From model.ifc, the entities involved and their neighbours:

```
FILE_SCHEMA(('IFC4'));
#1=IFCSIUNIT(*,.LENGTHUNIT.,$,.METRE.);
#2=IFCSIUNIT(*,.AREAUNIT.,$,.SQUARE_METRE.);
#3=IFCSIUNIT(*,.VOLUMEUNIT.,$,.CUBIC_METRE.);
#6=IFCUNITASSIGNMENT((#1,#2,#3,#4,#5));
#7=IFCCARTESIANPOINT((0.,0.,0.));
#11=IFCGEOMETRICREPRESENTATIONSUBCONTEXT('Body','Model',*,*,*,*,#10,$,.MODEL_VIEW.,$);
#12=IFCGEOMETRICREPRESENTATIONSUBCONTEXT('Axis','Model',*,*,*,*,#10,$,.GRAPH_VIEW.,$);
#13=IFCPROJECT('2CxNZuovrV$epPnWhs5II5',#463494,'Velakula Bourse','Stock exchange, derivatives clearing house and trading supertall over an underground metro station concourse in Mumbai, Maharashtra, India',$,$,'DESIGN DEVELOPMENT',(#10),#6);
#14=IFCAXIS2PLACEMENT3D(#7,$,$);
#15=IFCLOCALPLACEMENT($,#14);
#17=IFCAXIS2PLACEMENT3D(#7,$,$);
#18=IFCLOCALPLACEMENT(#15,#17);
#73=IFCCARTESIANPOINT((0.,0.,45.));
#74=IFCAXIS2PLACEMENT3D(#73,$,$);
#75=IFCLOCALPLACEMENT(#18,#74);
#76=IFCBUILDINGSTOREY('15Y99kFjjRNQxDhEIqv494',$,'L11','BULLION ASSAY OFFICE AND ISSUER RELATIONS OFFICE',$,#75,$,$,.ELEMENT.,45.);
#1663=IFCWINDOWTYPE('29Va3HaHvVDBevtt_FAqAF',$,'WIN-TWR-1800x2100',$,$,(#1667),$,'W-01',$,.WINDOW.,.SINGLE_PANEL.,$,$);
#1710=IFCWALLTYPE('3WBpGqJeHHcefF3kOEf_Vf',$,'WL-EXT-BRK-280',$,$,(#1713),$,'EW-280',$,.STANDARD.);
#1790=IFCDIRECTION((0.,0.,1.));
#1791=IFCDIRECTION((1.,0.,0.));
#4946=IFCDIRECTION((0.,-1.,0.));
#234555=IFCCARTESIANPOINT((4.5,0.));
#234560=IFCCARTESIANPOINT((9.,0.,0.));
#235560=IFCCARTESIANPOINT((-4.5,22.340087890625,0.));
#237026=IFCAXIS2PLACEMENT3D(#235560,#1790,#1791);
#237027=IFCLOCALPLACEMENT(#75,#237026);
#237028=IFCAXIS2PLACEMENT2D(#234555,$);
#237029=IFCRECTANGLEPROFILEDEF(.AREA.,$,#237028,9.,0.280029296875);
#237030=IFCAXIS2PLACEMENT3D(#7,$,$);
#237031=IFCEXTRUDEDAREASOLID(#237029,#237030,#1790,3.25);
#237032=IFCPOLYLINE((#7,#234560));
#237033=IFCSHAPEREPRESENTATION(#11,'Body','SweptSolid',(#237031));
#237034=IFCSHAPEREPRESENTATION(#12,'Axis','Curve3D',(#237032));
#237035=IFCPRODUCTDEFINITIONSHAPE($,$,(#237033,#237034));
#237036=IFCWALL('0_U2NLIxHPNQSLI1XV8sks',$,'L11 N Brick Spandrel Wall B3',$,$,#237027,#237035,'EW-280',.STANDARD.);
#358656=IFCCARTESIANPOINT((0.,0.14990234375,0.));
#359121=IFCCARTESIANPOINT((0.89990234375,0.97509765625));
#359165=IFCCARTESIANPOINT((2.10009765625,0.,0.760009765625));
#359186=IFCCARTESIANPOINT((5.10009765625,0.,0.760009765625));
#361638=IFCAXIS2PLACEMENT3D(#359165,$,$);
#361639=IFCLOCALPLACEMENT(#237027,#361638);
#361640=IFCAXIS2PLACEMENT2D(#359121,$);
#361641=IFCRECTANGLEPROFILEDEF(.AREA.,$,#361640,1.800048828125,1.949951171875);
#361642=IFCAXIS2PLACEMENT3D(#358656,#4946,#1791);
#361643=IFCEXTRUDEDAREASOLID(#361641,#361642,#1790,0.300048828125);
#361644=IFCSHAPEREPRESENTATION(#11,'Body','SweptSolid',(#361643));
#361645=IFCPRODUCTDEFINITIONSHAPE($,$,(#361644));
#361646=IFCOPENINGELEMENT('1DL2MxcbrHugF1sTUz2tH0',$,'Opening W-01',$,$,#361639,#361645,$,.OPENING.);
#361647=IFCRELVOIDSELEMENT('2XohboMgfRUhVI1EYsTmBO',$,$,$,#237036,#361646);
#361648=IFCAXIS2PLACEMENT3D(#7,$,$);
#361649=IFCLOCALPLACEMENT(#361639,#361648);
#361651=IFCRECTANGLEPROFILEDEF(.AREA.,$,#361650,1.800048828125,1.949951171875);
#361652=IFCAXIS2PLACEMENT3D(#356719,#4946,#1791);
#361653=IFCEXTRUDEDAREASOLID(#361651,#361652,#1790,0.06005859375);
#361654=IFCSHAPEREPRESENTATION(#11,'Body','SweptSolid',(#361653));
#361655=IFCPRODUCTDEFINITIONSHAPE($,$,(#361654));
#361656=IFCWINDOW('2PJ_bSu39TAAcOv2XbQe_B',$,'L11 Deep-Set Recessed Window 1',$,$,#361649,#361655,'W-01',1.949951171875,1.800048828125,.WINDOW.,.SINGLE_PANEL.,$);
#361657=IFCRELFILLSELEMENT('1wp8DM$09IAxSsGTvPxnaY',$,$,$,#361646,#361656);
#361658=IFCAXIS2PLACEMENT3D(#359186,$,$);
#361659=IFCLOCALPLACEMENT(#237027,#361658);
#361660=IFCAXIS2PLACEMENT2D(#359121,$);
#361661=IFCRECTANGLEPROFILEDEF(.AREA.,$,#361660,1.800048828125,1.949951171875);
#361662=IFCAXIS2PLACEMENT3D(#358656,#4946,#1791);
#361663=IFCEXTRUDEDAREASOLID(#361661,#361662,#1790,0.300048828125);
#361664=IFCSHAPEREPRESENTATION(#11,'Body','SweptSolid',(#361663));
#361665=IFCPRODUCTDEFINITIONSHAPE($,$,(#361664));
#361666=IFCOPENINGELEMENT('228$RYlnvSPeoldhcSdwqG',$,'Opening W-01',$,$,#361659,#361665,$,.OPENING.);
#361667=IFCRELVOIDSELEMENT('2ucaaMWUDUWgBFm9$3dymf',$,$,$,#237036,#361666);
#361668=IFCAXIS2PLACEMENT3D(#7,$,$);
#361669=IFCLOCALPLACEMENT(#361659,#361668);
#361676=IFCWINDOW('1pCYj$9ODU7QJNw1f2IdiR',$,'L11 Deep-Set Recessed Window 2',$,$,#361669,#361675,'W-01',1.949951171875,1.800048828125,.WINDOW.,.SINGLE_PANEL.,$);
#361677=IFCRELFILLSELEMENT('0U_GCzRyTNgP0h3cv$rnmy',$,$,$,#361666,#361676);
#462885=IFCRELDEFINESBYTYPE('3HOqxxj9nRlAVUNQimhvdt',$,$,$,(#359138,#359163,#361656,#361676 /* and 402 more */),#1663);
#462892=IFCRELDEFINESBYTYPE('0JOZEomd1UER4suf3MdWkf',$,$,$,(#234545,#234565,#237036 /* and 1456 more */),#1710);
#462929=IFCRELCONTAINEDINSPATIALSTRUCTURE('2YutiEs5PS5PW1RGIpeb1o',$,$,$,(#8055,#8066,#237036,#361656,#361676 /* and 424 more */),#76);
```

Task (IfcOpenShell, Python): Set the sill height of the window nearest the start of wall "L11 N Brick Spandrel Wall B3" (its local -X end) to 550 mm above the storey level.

```python
import numpy as np
import ifcopenshell
import ifcopenshell.api.geometry
import ifcopenshell.geom
import ifcopenshell.util.element
import ifcopenshell.util.placement
import ifcopenshell.util.shape
import ifcopenshell.util.unit

model = ifcopenshell.open("model.ifc")
unit_scale = ifcopenshell.util.unit.calculate_unit_scale(model)

window = model.by_id(361656)
opening = window.FillsVoids[0].RelatingOpeningElement
storey = ifcopenshell.util.element.get_container(window, ifc_class="IfcBuildingStorey")
level = ifcopenshell.util.placement.get_local_placement(storey.ObjectPlacement)[2, 3]

# The opening's origin need not be at the sill, so measure its lowest point.
shape = ifcopenshell.geom.create_shape(ifcopenshell.geom.settings(), opening)
bottom = ifcopenshell.util.shape.get_shape_bottom_elevation(shape, shape.geometry) / unit_scale
dz = level + 0.55 / unit_scale - bottom

shift = np.array([0.0, 0.0, dz])
# The window is placed relative to its opening, so it follows when the opening moves.
matrix = ifcopenshell.util.placement.get_local_placement(opening.ObjectPlacement)
matrix[:3, 3] += shift
ifcopenshell.api.geometry.edit_object_placement(
    model, product=opening, matrix=matrix, is_si=False, should_transform_children=True
)

print(f"moved by {dz * unit_scale:+.3f} m")

model.write("model_updated.ifc")
```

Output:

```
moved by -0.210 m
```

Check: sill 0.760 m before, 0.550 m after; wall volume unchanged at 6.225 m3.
